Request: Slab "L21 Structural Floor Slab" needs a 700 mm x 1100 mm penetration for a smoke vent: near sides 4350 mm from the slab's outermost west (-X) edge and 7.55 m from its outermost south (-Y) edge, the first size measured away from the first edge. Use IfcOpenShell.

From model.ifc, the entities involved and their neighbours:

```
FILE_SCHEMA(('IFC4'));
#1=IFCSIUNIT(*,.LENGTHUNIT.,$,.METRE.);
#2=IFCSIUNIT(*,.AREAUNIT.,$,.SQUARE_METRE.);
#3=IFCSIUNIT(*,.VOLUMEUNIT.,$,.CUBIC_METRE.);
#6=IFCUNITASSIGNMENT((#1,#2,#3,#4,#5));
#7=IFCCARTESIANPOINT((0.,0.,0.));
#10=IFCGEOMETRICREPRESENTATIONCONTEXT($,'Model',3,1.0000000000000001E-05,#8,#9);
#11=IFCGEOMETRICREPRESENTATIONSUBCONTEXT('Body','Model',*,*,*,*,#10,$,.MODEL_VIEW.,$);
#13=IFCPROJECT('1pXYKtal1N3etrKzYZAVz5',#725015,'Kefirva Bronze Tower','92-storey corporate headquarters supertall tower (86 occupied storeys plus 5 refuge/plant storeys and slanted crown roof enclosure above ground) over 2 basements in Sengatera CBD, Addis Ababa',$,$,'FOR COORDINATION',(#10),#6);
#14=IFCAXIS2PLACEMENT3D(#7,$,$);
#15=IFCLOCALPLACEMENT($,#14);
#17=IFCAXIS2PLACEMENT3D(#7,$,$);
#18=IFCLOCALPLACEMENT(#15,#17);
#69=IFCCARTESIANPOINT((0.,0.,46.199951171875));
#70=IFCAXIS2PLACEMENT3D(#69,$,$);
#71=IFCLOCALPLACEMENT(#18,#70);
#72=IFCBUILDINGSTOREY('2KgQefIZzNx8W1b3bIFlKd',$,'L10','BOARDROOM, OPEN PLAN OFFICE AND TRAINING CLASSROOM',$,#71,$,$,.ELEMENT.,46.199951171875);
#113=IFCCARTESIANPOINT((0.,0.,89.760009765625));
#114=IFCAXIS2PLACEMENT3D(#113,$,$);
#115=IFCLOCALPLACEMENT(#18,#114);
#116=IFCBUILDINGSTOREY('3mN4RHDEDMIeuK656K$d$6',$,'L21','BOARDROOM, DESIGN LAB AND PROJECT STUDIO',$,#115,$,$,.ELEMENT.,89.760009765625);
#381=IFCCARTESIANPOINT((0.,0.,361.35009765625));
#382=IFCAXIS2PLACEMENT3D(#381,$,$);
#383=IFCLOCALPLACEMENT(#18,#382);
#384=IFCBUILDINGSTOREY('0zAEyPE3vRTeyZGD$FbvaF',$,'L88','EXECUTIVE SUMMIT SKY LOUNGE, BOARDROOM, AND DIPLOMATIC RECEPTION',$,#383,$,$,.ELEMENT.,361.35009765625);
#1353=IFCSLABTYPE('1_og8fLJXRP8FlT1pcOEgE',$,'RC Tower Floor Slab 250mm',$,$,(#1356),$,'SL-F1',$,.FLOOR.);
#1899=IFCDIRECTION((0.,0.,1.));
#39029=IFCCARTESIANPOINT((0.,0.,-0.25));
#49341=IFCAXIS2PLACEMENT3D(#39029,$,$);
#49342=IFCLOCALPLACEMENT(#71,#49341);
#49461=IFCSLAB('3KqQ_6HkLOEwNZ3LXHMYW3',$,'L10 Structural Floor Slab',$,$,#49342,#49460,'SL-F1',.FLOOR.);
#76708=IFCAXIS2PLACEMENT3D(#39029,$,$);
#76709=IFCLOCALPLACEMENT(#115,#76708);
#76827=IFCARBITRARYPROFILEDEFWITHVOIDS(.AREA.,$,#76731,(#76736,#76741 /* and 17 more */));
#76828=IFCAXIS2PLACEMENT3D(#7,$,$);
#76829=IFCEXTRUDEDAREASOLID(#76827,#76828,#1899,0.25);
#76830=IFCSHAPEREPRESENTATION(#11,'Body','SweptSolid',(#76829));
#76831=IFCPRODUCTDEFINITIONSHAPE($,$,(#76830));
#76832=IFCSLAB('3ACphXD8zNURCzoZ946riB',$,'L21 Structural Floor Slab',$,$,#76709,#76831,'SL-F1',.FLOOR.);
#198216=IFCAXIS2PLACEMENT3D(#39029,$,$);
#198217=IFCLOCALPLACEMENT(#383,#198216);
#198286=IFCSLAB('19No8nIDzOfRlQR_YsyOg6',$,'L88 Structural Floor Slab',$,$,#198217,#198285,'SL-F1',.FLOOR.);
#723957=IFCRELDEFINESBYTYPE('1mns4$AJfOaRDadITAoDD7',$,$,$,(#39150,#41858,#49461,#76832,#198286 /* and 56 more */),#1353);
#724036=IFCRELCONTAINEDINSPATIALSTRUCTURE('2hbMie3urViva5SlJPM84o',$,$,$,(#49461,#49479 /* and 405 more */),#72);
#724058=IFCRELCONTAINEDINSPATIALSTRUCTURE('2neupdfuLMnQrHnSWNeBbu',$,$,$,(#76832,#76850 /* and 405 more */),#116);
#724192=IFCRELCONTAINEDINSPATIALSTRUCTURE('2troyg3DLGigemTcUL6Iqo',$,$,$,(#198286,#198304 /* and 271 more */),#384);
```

```python
import numpy as np
import ifcopenshell
import ifcopenshell.api.feature
import ifcopenshell.api.geometry
import ifcopenshell.api.root
import ifcopenshell.geom
import ifcopenshell.util.placement
import ifcopenshell.util.representation
import ifcopenshell.util.shape
import ifcopenshell.util.unit

model = ifcopenshell.open("model.ifc")
unit_scale = ifcopenshell.util.unit.calculate_unit_scale(model)
settings = ifcopenshell.geom.settings()


def volume(element):
    """Net volume in cubic metres, openings subtracted."""
    shape = ifcopenshell.geom.create_shape(settings, element)
    return ifcopenshell.util.shape.get_volume(shape.geometry)


slab = model.by_guid("3ACphXD8zNURCzoZ946riB")
before = volume(slab)

# Extent in the slab's own axes, in metres. The edges named are its -X and -Y sides.
slab_shape = ifcopenshell.geom.create_shape(settings, slab)
vertices = ifcopenshell.util.shape.get_vertices(slab_shape.geometry)
x_min, y_min, bottom = vertices.min(axis=0)
top = vertices[:, 2].max()

opening = ifcopenshell.api.root.create_entity(model, ifc_class="IfcOpeningElement", name="Smoke vent opening", predefined_type="OPENING")
context = ifcopenshell.util.representation.get_context(model, "Model", "Body", "MODEL_VIEW")
width, depth = 0.7, 1.1
outline = [(0.0, 0.0), (width, 0.0), (width, depth), (0.0, depth), (0.0, 0.0)]
# Overshoot both faces by 50 mm so the cut is clean.
shape = ifcopenshell.api.geometry.add_slab_representation(
    model, context=context, depth=top - bottom + 0.1, polyline=outline
)
ifcopenshell.api.geometry.assign_representation(model, product=opening, representation=shape)

matrix = ifcopenshell.util.placement.get_local_placement(slab.ObjectPlacement)
matrix[:, 3] = matrix @ np.append(np.array([x_min + 4.35, y_min + 7.55, bottom - 0.05]) / unit_scale, 1.0)
ifcopenshell.api.geometry.edit_object_placement(model, product=opening, matrix=matrix, is_si=False)
ifcopenshell.api.feature.add_feature(model, feature=opening, element=slab)

after = volume(slab)

print(f"slab volume {before:.3f} -> {after:.3f} m3")

model.write("model_edited.ifc")
```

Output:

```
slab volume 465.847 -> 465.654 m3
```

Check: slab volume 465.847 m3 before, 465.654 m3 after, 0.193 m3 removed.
